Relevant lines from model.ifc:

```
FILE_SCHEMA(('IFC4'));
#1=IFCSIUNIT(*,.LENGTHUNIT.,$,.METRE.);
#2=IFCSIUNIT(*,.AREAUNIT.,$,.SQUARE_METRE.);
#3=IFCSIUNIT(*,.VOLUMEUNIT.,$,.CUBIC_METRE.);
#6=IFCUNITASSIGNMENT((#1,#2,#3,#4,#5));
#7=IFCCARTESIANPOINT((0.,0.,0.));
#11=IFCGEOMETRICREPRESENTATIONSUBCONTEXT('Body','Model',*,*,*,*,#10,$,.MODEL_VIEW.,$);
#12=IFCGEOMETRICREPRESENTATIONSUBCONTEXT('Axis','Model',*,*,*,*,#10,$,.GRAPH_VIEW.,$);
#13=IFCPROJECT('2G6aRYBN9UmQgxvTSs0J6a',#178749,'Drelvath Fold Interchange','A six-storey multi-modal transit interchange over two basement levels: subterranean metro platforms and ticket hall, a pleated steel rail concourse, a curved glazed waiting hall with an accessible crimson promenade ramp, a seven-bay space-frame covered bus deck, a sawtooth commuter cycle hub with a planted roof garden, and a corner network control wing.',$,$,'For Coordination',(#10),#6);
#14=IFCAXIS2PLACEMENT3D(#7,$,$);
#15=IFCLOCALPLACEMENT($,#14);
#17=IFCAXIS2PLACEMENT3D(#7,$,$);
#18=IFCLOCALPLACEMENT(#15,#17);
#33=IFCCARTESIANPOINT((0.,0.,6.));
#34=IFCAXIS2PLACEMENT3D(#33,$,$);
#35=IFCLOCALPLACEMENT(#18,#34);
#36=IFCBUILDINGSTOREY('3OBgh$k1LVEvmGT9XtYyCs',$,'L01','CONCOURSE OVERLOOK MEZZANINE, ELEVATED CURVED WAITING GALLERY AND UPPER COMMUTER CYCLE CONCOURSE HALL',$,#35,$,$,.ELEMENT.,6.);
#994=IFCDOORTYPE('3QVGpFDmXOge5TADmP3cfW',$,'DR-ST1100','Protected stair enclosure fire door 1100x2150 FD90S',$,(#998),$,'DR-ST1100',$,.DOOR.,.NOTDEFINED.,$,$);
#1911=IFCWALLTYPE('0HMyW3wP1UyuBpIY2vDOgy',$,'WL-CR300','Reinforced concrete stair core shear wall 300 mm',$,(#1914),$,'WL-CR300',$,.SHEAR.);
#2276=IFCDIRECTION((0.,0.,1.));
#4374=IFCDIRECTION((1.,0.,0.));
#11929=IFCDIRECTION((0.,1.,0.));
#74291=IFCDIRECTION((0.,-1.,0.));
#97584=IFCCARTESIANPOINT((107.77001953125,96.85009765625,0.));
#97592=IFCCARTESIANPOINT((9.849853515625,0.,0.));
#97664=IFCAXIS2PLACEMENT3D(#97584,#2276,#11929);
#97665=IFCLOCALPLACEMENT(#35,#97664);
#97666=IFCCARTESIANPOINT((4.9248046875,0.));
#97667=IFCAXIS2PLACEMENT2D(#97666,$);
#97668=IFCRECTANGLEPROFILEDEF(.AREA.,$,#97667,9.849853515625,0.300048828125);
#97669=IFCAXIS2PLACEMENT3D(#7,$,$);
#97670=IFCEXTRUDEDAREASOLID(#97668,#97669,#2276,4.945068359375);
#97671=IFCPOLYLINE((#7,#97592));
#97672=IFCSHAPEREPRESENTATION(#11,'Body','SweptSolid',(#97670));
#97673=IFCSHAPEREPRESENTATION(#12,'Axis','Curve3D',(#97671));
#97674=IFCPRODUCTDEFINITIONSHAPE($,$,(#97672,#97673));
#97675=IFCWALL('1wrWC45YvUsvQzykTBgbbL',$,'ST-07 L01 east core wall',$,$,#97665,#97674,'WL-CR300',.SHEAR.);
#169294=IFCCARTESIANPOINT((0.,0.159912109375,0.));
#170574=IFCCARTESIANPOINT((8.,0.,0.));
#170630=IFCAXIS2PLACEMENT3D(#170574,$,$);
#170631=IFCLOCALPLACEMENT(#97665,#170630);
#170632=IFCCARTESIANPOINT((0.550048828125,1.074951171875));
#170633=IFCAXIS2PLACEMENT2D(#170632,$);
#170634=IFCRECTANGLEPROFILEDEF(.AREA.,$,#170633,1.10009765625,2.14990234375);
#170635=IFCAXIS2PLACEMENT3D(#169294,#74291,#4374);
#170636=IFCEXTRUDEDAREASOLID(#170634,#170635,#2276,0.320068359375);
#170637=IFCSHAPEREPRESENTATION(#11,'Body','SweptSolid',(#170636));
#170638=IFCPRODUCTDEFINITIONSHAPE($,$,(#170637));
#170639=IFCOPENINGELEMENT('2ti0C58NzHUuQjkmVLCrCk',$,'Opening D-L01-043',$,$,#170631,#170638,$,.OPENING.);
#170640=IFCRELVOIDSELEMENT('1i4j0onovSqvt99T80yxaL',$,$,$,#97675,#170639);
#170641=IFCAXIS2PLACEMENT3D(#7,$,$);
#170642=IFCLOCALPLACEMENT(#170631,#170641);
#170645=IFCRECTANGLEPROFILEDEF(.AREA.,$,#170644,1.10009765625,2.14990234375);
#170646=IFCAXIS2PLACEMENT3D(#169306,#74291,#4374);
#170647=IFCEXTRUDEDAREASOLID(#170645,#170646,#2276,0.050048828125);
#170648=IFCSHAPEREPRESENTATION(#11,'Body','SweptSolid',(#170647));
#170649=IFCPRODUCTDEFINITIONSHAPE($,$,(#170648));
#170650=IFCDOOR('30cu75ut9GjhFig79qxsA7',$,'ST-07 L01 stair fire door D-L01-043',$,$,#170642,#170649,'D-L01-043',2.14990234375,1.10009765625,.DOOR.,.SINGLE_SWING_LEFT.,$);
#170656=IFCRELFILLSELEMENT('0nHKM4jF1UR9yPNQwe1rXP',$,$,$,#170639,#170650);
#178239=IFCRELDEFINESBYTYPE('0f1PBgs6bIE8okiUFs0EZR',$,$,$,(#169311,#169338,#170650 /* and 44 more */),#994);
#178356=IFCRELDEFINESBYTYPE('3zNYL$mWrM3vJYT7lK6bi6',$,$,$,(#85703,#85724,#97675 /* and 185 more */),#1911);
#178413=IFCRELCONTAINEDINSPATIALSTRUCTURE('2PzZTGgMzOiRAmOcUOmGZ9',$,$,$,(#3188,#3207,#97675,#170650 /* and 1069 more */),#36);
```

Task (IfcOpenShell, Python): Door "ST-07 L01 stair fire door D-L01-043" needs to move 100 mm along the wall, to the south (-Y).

```python
import ifcopenshell
import ifcopenshell.api.geometry
import ifcopenshell.util.placement

model = ifcopenshell.open("model.ifc")

door = model.by_guid("30cu75ut9GjhFig79qxsA7")
opening = door.FillsVoids[0].RelatingOpeningElement
wall = opening.VoidsElements[0].RelatingBuildingElement

wall_matrix = ifcopenshell.util.placement.get_local_placement(wall.ObjectPlacement)
shift = wall_matrix[:3, 0] * -0.1
before = ifcopenshell.util.placement.get_local_placement(door.ObjectPlacement)[:3, 3].copy()

# The door is placed relative to its opening, so it follows when the opening moves.
matrix = ifcopenshell.util.placement.get_local_placement(opening.ObjectPlacement)
matrix[:3, 3] += shift
ifcopenshell.api.geometry.edit_object_placement(
    model, product=opening, matrix=matrix, is_si=False, should_transform_children=True
)

after = ifcopenshell.util.placement.get_local_placement(door.ObjectPlacement)[:3, 3]
print("door moved by", (after - before).round(3) + 0.0)

model.write("model-out.ifc")
```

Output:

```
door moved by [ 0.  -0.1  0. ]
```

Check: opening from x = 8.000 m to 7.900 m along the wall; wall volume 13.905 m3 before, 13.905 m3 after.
